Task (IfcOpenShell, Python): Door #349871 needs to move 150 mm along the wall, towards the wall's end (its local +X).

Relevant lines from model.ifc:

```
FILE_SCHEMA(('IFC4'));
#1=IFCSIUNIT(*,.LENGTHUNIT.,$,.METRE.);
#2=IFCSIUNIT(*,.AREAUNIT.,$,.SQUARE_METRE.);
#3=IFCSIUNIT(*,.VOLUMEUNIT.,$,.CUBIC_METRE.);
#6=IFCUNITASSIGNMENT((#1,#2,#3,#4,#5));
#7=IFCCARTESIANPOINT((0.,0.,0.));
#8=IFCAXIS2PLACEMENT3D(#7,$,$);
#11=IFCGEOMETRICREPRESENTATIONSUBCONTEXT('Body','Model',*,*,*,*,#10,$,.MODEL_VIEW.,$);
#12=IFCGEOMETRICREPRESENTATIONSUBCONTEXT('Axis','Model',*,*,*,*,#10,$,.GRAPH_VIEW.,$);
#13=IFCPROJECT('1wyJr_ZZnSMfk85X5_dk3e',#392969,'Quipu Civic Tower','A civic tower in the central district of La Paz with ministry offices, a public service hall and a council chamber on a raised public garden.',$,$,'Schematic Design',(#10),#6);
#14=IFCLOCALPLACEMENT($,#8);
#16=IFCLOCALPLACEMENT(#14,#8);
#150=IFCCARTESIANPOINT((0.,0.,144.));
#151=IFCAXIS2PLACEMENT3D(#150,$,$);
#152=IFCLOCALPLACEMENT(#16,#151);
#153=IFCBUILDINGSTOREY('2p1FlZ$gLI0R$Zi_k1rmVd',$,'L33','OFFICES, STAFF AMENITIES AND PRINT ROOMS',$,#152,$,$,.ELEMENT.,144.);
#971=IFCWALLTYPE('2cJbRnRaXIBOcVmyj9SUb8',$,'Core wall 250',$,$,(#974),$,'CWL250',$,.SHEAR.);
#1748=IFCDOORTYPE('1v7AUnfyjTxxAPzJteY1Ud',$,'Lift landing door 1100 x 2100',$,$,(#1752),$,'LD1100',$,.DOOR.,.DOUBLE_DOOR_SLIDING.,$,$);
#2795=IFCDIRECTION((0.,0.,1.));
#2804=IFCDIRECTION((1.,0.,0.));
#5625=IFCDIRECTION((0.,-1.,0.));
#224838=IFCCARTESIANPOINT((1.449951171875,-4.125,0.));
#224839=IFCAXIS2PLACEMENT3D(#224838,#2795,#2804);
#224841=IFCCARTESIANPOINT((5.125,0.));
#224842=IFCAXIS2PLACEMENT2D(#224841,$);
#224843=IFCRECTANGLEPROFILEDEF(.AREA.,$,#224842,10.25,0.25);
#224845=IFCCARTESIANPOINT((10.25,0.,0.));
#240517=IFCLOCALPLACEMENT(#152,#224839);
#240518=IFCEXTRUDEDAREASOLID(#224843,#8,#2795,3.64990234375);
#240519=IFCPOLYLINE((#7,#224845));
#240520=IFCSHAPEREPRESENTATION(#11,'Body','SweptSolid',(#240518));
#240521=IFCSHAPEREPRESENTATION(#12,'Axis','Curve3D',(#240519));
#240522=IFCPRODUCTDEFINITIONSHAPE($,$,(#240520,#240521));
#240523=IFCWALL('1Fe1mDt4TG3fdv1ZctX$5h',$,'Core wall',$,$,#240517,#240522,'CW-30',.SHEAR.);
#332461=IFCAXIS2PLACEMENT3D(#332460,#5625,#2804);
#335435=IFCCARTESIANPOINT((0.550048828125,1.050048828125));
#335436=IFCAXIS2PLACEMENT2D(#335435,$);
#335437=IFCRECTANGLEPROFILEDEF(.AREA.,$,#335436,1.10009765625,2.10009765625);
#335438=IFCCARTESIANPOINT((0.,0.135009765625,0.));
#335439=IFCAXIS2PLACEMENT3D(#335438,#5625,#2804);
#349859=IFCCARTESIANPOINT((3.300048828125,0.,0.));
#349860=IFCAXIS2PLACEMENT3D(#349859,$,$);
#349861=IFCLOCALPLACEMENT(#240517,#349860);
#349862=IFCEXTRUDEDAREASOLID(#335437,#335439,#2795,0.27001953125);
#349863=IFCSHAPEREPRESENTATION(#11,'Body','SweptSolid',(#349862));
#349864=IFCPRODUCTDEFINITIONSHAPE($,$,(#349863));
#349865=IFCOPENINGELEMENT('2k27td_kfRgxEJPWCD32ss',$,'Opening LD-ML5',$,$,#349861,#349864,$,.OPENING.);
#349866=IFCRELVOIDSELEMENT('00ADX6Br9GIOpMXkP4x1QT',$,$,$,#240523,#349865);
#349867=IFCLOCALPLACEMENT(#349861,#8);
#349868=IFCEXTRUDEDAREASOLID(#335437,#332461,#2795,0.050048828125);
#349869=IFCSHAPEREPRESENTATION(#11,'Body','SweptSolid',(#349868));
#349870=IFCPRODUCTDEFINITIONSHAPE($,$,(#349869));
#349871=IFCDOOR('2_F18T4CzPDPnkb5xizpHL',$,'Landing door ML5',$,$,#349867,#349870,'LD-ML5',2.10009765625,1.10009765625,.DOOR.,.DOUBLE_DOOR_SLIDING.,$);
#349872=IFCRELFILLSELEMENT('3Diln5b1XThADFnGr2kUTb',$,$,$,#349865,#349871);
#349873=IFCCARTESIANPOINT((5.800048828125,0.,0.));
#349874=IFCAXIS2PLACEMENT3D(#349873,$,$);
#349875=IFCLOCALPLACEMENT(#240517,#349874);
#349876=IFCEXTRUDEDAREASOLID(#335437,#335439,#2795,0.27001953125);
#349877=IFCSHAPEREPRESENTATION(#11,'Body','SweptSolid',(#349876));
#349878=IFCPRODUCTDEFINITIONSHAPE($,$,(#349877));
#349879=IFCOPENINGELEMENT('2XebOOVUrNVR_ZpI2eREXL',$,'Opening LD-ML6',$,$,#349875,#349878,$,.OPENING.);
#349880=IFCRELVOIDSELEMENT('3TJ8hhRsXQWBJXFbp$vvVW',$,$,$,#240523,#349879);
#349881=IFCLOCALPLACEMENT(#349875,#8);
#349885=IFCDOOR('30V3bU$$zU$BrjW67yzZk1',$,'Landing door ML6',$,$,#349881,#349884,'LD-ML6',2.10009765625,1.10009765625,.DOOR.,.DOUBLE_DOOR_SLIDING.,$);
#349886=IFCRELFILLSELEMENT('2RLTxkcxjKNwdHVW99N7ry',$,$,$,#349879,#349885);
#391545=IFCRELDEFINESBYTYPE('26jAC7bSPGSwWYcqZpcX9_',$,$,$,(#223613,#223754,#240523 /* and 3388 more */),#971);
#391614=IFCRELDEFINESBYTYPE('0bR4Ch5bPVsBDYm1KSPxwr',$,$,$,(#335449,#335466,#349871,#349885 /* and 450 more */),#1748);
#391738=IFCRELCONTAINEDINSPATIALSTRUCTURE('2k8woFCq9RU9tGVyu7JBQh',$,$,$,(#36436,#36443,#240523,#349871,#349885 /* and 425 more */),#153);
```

```python
import ifcopenshell
import ifcopenshell.api.geometry
import ifcopenshell.util.placement
import ifcopenshell.util.unit

model = ifcopenshell.open("model.ifc")
unit_scale = ifcopenshell.util.unit.calculate_unit_scale(model)

door = model.by_guid("2_F18T4CzPDPnkb5xizpHL")
opening = door.FillsVoids[0].RelatingOpeningElement
wall = opening.VoidsElements[0].RelatingBuildingElement

wall_matrix = ifcopenshell.util.placement.get_local_placement(wall.ObjectPlacement)
shift = wall_matrix[:3, 0] * 0.15 / unit_scale
before = ifcopenshell.util.placement.get_local_placement(door.ObjectPlacement)[:3, 3].copy()

# The door is placed relative to its opening, so it follows when the opening moves.
matrix = ifcopenshell.util.placement.get_local_placement(opening.ObjectPlacement)
matrix[:3, 3] += shift
ifcopenshell.api.geometry.edit_object_placement(
    model, product=opening, matrix=matrix, is_si=False, should_transform_children=True
)

after = ifcopenshell.util.placement.get_local_placement(door.ObjectPlacement)[:3, 3]
print("door moved by", (after - before).round(3) + 0.0)

model.write("model_edited.ifc")
```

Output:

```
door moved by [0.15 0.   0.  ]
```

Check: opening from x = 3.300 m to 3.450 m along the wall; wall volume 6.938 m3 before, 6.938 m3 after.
